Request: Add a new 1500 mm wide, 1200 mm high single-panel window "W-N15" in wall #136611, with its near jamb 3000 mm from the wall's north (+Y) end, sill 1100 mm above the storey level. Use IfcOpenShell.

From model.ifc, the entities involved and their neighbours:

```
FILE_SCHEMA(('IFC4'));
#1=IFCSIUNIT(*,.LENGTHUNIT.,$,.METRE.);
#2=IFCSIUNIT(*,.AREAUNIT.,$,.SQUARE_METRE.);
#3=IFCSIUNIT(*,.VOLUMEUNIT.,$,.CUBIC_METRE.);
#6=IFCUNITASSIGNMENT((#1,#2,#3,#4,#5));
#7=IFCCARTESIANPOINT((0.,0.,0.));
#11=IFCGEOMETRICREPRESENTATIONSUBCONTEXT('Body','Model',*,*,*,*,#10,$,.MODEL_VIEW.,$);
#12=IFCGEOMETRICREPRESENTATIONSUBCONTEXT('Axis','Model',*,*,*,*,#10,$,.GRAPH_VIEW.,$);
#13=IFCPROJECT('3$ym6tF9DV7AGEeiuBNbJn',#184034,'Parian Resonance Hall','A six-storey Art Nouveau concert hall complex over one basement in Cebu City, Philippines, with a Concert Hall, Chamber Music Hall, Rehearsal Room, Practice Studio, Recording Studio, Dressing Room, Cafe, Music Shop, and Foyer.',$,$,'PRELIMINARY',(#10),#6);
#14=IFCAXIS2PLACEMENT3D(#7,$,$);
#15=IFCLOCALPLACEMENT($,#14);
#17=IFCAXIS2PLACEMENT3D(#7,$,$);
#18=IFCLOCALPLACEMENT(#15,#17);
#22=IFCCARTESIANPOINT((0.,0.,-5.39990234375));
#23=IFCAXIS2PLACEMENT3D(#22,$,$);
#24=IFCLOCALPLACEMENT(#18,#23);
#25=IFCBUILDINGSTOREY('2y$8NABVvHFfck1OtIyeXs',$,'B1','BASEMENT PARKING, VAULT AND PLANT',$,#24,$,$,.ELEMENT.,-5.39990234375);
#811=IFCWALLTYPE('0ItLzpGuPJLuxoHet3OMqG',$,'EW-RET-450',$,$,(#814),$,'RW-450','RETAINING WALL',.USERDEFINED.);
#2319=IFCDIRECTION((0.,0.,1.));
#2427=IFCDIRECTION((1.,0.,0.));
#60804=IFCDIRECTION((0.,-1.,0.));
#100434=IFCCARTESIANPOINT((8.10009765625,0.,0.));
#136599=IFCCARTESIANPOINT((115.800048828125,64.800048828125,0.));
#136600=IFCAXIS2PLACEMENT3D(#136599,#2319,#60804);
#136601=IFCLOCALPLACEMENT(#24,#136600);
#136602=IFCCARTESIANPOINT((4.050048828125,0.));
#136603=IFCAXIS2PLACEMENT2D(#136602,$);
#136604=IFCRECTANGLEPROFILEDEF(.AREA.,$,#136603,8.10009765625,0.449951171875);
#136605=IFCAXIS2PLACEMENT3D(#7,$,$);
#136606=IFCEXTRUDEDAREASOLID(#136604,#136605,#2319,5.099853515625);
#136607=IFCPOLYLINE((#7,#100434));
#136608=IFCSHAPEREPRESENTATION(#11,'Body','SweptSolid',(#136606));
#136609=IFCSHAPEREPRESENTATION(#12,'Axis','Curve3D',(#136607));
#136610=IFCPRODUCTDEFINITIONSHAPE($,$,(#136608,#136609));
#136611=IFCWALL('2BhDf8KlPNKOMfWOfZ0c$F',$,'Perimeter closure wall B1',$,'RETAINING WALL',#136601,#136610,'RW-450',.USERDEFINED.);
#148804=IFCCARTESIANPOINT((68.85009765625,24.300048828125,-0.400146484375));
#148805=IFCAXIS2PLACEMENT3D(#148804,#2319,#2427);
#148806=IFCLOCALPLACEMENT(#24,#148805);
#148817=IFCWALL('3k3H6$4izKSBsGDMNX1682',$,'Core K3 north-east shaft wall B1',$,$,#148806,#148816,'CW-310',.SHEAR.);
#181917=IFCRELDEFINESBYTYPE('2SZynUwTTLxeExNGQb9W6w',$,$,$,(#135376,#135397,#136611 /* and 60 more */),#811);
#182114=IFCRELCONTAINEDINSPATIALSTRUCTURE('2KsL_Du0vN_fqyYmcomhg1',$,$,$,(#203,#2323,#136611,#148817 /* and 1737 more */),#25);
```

```python
import numpy as np
import ifcopenshell
import ifcopenshell.api.feature
import ifcopenshell.api.geometry
import ifcopenshell.api.root
import ifcopenshell.api.spatial
import ifcopenshell.geom
import ifcopenshell.util.element
import ifcopenshell.util.placement
import ifcopenshell.util.representation
import ifcopenshell.util.shape
import ifcopenshell.util.unit

model = ifcopenshell.open("model.ifc")
unit_scale = ifcopenshell.util.unit.calculate_unit_scale(model)
settings = ifcopenshell.geom.settings()


def volume(element):
    """Net volume in cubic metres, openings subtracted."""
    shape = ifcopenshell.geom.create_shape(settings, element)
    return ifcopenshell.util.shape.get_volume(shape.geometry)


wall = model.by_guid("2BhDf8KlPNKOMfWOfZ0c$F")
storey = ifcopenshell.util.element.get_container(wall, ifc_class="IfcBuildingStorey")
context = ifcopenshell.util.representation.get_context(model, "Model", "Body", "MODEL_VIEW")
before = volume(wall)

width, height, from_end, sill = 1.5, 1.2, 3, 1.1  # metres

# The wall runs along its own X axis, and the end named is its -X end.
wall_shape = ifcopenshell.geom.create_shape(settings, wall)
x, y, z = ifcopenshell.util.shape.get_vertices(wall_shape.geometry).T
start = x.min() + from_end
face, thickness = float(y.min()), float(y.max() - y.min())
wall_matrix = ifcopenshell.util.placement.get_local_placement(wall.ObjectPlacement)
level = ifcopenshell.util.placement.get_local_placement(storey.ObjectPlacement)[2, 3]


def in_wall(x, y):
    """Placement at x, y metres in the wall's axes, at sill height."""
    matrix = wall_matrix.copy()
    matrix[:, 3] = wall_matrix @ np.array([x / unit_scale, y / unit_scale, 0.0, 1.0])
    matrix[2, 3] = level + sill / unit_scale
    return matrix


# Opening: a box that overshoots both wall faces by 50 mm.
opening = ifcopenshell.api.root.create_entity(model, ifc_class="IfcOpeningElement", predefined_type="OPENING")
box = ifcopenshell.api.geometry.add_wall_representation(
    model, context=context, length=width, height=height, thickness=thickness + 0.1
)
ifcopenshell.api.geometry.assign_representation(model, product=opening, representation=box)
ifcopenshell.api.geometry.edit_object_placement(model, product=opening, matrix=in_wall(start, face - 0.05), is_si=False)
ifcopenshell.api.feature.add_feature(model, feature=opening, element=wall)

window = ifcopenshell.api.root.create_entity(model, ifc_class="IfcWindow", name="W-N15", predefined_type="WINDOW")
window.OverallWidth, window.OverallHeight = width / unit_scale, height / unit_scale
window.PartitioningType = "SINGLE_PANEL"
body = ifcopenshell.api.geometry.add_window_representation(
    model,
    context=context,
    overall_width=window.OverallWidth,
    overall_height=window.OverallHeight,
    partition_type="SINGLE_PANEL",
)
ifcopenshell.api.geometry.assign_representation(model, product=window, representation=body)
ifcopenshell.api.spatial.assign_container(model, products=[window], relating_structure=storey)
ifcopenshell.api.feature.add_filling(model, opening=opening, element=window)

# Centre the window in the wall's thickness.
ifcopenshell.api.geometry.edit_object_placement(model, product=window, matrix=in_wall(start, face), is_si=False)
window_shape = ifcopenshell.geom.create_shape(settings, window)
depth = ifcopenshell.util.shape.get_vertices(window_shape.geometry)[:, 1]
offset = face + thickness / 2 - (depth.min() + depth.max()) / 2
ifcopenshell.api.geometry.edit_object_placement(model, product=window, matrix=in_wall(start, offset), is_si=False)

after = volume(wall)

print(f"wall volume {before:.3f} -> {after:.3f} m3")

model.write("model_edited.ifc")
```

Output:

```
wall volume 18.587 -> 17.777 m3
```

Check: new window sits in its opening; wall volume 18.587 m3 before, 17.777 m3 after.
